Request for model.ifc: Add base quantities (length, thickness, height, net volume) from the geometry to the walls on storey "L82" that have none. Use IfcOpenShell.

First a look at what the model holds.

```python
import ifcopenshell
import ifcopenshell.util.element
import ifcopenshell.util.unit

model = ifcopenshell.open("model.ifc")
print(model.schema)
for unit_type in ("LENGTHUNIT", "AREAUNIT", "VOLUMEUNIT"):
    print(unit_type, ifcopenshell.util.unit.calculate_unit_scale(model, unit_type))
storey = next(s for s in model.by_type("IfcBuildingStorey") if s.Name == "L82")
walls = [e for e in ifcopenshell.util.element.get_decomposition(storey) if e.is_a("IfcWall")]
for e in sorted(walls, key=lambda e: e.id()):
    print(e.id(), e.is_a(), e.Name, list(ifcopenshell.util.element.get_psets(e, qtos_only=True)), sep=" | ")
```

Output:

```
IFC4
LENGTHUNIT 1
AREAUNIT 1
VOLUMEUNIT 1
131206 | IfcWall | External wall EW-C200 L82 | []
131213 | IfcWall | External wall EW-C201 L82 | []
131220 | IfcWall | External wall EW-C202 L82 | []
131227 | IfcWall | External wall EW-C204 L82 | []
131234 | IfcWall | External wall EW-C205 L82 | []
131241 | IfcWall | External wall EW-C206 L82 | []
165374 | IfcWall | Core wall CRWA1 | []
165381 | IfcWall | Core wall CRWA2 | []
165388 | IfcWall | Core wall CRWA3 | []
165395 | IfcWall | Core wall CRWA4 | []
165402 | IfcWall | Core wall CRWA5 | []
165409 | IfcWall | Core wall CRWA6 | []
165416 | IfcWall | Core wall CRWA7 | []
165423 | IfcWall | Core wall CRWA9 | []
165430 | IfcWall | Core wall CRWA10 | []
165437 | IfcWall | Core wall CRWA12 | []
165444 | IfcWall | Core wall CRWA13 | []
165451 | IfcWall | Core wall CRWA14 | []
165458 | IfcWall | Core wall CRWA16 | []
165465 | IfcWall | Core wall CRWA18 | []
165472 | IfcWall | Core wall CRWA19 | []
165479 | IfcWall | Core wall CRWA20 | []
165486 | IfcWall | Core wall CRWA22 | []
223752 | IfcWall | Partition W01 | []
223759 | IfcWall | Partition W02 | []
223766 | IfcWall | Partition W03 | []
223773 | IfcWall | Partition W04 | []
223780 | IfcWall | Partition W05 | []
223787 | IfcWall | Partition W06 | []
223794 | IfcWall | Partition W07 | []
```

```python
import ifcopenshell
import ifcopenshell.api.pset
import ifcopenshell.geom
import ifcopenshell.util.element
import ifcopenshell.util.shape
import ifcopenshell.util.unit

model = ifcopenshell.open("model.ifc")
unit_scale = ifcopenshell.util.unit.calculate_unit_scale(model)
volume_scale = ifcopenshell.util.unit.calculate_unit_scale(model, "VOLUMEUNIT")
settings = ifcopenshell.geom.settings()

storey = next(s for s in model.by_type("IfcBuildingStorey") if s.Name == "L82")
walls = [e for e in ifcopenshell.util.element.get_decomposition(storey) if e.is_a("IfcWall")]

for e in sorted(walls, key=lambda e: e.id()):
    if ifcopenshell.util.element.get_psets(e, qtos_only=True, should_inherit=False):
        continue
    # Geometry comes back in metres, in the element's own axes.
    shape = ifcopenshell.geom.create_shape(settings, e)
    values = {
        "Length": ifcopenshell.util.shape.get_x(shape.geometry) / unit_scale,
        "Width": ifcopenshell.util.shape.get_y(shape.geometry) / unit_scale,
        "Height": ifcopenshell.util.shape.get_z(shape.geometry) / unit_scale,
        "NetVolume": ifcopenshell.util.shape.get_volume(shape.geometry) / volume_scale,
    }
    qto = ifcopenshell.api.pset.add_qto(model, product=e, name="Qto_WallBaseQuantities")
    ifcopenshell.api.pset.edit_qto(model, qto=qto, properties=values)
    print(e.id(), {k: round(v, 3) for k, v in values.items()})

model.write("model-out.ifc")
```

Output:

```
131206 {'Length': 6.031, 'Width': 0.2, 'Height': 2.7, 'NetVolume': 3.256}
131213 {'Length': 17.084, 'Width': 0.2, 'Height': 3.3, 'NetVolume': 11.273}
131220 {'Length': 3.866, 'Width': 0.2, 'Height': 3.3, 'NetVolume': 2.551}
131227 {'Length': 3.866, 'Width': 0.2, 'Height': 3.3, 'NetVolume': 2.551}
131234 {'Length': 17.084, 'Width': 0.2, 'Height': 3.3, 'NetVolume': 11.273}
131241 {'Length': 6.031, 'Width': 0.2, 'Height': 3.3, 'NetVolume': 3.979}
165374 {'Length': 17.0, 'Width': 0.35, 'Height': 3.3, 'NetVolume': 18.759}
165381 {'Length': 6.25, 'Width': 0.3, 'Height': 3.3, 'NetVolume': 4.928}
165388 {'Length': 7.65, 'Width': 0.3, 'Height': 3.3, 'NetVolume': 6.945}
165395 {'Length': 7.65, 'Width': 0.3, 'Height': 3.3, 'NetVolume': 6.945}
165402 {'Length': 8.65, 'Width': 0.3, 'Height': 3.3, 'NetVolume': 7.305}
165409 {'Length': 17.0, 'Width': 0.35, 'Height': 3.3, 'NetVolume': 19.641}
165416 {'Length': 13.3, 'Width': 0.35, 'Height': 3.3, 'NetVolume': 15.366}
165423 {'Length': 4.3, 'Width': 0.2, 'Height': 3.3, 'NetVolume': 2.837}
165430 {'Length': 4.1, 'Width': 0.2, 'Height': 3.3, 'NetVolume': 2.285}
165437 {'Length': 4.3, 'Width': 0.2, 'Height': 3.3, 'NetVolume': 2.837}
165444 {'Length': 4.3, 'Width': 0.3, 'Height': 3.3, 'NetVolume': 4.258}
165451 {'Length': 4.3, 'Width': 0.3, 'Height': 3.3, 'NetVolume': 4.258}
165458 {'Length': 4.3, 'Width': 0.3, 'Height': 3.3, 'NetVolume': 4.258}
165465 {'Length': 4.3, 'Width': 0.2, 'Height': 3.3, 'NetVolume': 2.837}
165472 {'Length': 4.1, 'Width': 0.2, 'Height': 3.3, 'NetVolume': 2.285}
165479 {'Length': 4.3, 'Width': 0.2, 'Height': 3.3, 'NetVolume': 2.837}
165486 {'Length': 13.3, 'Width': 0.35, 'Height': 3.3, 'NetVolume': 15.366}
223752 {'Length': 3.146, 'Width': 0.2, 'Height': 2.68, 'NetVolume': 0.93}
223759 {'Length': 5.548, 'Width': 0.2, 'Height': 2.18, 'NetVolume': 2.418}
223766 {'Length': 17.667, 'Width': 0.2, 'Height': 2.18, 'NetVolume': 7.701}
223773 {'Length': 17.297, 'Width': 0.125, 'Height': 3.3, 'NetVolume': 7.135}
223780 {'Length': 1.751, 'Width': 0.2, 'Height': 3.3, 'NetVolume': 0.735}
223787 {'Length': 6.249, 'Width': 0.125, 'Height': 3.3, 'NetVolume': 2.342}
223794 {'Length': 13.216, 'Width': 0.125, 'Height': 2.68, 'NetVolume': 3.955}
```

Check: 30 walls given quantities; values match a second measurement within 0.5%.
